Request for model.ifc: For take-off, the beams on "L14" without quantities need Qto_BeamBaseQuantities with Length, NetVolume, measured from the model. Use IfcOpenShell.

First a look at what the model holds.

```python
import ifcopenshell
import ifcopenshell.util.element
import ifcopenshell.util.unit

model = ifcopenshell.open("model.ifc")
print(model.schema)
for unit_type in ("LENGTHUNIT", "AREAUNIT", "VOLUMEUNIT"):
    print(unit_type, ifcopenshell.util.unit.calculate_unit_scale(model, unit_type))
storey = next(s for s in model.by_type("IfcBuildingStorey") if s.Name == "L14")
beams = [e for e in ifcopenshell.util.element.get_decomposition(storey) if e.is_a("IfcBeam")]
for e in sorted(beams, key=lambda e: e.id()):
    print(e.id(), e.is_a(), e.Name, list(ifcopenshell.util.element.get_psets(e, qtos_only=True)), sep=" | ")
```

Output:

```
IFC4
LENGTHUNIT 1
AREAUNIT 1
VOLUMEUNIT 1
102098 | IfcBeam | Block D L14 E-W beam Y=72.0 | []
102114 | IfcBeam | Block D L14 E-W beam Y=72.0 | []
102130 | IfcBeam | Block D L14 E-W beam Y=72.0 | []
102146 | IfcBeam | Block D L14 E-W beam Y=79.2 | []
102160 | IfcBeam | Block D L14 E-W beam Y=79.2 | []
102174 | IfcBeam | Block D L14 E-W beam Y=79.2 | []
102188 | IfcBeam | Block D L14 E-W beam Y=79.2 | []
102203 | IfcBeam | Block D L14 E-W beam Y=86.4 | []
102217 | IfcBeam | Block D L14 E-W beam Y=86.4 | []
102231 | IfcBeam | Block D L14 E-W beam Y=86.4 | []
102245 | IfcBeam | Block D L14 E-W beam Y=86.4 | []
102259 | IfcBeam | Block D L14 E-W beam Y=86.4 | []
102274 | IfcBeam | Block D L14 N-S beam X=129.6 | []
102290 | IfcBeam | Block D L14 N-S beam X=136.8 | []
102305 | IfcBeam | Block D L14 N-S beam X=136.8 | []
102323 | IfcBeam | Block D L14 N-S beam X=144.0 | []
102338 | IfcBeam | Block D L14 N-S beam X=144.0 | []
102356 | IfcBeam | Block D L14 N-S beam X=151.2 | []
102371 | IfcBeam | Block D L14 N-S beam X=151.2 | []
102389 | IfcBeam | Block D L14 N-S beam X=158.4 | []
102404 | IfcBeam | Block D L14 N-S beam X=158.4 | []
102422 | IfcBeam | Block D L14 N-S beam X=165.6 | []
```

```python
import ifcopenshell
import ifcopenshell.api.pset
import ifcopenshell.geom
import ifcopenshell.util.element
import ifcopenshell.util.shape
import ifcopenshell.util.unit

model = ifcopenshell.open("model.ifc")
unit_scale = ifcopenshell.util.unit.calculate_unit_scale(model)
volume_scale = ifcopenshell.util.unit.calculate_unit_scale(model, "VOLUMEUNIT")
settings = ifcopenshell.geom.settings()

storey = next(s for s in model.by_type("IfcBuildingStorey") if s.Name == "L14")
beams = [e for e in ifcopenshell.util.element.get_decomposition(storey) if e.is_a("IfcBeam")]

for e in sorted(beams, key=lambda e: e.id()):
    if ifcopenshell.util.element.get_psets(e, qtos_only=True, should_inherit=False):
        continue
    # Geometry comes back in metres, in the element's own axes.
    shape = ifcopenshell.geom.create_shape(settings, e)
    values = {
        "Length": ifcopenshell.util.shape.get_max_xyz(shape.geometry) / unit_scale,
        "NetVolume": ifcopenshell.util.shape.get_volume(shape.geometry) / volume_scale,
    }
    qto = ifcopenshell.api.pset.add_qto(model, product=e, name="Qto_BeamBaseQuantities")
    ifcopenshell.api.pset.edit_qto(model, qto=qto, properties=values)
    print(e.id(), {k: round(v, 3) for k, v in values.items()})

model.write("model_updated.ifc")
```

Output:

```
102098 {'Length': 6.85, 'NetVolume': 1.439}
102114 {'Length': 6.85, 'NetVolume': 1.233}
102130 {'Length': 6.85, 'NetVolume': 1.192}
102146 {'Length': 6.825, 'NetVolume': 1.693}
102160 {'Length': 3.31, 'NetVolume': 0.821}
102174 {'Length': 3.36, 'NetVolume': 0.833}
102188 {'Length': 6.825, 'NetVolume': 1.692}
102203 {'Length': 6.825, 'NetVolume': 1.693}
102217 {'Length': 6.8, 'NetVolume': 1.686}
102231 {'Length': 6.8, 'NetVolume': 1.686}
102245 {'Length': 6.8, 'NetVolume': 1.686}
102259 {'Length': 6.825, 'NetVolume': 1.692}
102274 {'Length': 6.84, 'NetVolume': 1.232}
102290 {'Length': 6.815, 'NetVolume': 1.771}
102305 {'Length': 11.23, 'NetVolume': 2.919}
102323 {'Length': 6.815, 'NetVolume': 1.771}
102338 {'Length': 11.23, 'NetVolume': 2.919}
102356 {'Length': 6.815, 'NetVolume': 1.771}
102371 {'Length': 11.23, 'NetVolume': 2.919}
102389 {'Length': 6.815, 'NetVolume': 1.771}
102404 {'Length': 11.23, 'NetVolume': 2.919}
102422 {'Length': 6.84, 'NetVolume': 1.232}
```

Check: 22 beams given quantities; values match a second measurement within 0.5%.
